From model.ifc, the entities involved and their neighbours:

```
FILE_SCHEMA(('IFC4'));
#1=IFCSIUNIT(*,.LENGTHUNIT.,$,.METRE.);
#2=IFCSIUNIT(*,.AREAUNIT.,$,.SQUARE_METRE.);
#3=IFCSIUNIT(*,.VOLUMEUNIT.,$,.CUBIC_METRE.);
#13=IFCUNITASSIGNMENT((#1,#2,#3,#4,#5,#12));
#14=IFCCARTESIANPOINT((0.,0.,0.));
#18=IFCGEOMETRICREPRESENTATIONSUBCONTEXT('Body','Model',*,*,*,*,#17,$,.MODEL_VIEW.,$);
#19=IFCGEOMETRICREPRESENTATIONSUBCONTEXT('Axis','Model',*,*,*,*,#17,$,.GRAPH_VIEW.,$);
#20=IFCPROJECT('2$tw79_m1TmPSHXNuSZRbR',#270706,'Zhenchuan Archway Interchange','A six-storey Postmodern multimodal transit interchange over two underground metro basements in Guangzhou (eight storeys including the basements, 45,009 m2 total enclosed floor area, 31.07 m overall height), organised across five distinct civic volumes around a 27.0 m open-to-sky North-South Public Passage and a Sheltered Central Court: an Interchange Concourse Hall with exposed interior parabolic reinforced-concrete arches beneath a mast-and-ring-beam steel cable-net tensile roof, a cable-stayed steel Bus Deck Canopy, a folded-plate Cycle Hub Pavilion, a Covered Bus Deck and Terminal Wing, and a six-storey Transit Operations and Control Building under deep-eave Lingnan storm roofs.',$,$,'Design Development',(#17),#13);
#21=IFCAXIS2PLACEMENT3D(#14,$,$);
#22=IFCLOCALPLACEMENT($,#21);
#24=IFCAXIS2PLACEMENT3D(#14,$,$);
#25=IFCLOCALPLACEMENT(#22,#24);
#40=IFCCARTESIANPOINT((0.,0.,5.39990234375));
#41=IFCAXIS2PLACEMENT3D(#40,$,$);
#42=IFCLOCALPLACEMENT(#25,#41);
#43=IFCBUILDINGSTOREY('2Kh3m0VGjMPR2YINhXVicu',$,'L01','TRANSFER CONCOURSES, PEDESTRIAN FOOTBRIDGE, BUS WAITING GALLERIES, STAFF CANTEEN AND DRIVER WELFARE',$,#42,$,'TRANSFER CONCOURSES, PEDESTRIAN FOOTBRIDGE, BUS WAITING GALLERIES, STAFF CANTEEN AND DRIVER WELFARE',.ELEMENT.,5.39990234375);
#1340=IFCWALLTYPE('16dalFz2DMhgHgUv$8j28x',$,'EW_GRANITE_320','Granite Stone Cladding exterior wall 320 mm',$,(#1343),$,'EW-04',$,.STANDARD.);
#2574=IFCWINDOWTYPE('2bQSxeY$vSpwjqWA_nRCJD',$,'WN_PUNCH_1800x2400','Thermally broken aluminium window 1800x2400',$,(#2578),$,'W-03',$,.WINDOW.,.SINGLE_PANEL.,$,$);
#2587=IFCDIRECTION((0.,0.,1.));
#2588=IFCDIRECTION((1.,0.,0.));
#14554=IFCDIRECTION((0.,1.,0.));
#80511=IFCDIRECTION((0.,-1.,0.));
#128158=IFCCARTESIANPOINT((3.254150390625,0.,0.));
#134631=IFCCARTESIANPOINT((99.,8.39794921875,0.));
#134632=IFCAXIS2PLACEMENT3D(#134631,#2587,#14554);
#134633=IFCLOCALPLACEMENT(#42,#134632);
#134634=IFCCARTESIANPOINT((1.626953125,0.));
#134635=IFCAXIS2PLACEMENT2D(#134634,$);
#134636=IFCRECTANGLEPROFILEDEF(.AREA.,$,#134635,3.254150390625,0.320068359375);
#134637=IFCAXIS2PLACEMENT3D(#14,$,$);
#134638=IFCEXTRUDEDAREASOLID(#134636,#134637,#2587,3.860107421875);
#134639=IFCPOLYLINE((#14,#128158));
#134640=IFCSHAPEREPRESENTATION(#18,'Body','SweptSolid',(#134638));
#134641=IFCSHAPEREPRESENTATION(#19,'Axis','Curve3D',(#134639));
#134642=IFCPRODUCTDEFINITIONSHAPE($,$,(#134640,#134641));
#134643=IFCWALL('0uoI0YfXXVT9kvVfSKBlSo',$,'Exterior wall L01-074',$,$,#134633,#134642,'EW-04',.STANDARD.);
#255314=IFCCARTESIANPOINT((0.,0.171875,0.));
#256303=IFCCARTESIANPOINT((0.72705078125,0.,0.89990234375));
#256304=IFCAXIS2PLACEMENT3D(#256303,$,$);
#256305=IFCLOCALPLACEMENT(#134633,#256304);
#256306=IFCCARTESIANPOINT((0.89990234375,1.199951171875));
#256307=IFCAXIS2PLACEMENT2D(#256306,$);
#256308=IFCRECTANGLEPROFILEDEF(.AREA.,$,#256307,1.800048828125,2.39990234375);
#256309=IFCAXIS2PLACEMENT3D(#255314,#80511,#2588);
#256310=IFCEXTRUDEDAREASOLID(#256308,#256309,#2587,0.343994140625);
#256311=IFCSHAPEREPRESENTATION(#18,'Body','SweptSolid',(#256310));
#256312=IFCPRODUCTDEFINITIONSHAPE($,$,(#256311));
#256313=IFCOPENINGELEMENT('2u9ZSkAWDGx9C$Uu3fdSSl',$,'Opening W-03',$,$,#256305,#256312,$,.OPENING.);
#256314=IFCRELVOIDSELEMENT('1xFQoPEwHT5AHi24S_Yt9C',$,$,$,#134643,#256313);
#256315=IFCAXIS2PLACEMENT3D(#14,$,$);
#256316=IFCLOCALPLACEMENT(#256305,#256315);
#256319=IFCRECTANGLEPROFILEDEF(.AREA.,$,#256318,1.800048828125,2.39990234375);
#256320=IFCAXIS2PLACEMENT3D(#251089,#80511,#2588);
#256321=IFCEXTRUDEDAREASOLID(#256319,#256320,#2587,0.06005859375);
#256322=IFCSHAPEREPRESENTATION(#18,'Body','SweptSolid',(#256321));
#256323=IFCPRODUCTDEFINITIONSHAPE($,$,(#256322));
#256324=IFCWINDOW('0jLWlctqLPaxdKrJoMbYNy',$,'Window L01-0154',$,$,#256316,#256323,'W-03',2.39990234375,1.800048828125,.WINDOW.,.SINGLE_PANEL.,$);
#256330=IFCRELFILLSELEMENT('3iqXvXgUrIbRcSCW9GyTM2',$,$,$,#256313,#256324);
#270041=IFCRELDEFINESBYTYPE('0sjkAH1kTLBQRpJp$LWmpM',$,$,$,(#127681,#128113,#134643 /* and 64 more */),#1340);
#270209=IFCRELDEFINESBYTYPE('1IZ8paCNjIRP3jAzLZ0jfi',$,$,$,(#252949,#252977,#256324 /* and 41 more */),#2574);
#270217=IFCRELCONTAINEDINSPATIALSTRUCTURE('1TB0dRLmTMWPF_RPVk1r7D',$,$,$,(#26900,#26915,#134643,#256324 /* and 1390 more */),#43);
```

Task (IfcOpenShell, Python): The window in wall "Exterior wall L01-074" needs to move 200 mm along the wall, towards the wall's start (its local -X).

```python
import ifcopenshell
import ifcopenshell.api.geometry
import ifcopenshell.util.placement

model = ifcopenshell.open("model.ifc")

window = model.by_guid("0jLWlctqLPaxdKrJoMbYNy")
opening = window.FillsVoids[0].RelatingOpeningElement
wall = opening.VoidsElements[0].RelatingBuildingElement

wall_matrix = ifcopenshell.util.placement.get_local_placement(wall.ObjectPlacement)
shift = wall_matrix[:3, 0] * -0.2
before = ifcopenshell.util.placement.get_local_placement(window.ObjectPlacement)[:3, 3].copy()

# The window is placed relative to its opening, so it follows when the opening moves.
matrix = ifcopenshell.util.placement.get_local_placement(opening.ObjectPlacement)
matrix[:3, 3] += shift
ifcopenshell.api.geometry.edit_object_placement(
    model, product=opening, matrix=matrix, is_si=False, should_transform_children=True
)

after = ifcopenshell.util.placement.get_local_placement(window.ObjectPlacement)[:3, 3]
print("window moved by", (after - before).round(3) + 0.0)

model.write("model_v2.ifc")
```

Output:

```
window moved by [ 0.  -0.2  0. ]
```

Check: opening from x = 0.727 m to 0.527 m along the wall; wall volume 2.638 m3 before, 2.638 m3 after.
